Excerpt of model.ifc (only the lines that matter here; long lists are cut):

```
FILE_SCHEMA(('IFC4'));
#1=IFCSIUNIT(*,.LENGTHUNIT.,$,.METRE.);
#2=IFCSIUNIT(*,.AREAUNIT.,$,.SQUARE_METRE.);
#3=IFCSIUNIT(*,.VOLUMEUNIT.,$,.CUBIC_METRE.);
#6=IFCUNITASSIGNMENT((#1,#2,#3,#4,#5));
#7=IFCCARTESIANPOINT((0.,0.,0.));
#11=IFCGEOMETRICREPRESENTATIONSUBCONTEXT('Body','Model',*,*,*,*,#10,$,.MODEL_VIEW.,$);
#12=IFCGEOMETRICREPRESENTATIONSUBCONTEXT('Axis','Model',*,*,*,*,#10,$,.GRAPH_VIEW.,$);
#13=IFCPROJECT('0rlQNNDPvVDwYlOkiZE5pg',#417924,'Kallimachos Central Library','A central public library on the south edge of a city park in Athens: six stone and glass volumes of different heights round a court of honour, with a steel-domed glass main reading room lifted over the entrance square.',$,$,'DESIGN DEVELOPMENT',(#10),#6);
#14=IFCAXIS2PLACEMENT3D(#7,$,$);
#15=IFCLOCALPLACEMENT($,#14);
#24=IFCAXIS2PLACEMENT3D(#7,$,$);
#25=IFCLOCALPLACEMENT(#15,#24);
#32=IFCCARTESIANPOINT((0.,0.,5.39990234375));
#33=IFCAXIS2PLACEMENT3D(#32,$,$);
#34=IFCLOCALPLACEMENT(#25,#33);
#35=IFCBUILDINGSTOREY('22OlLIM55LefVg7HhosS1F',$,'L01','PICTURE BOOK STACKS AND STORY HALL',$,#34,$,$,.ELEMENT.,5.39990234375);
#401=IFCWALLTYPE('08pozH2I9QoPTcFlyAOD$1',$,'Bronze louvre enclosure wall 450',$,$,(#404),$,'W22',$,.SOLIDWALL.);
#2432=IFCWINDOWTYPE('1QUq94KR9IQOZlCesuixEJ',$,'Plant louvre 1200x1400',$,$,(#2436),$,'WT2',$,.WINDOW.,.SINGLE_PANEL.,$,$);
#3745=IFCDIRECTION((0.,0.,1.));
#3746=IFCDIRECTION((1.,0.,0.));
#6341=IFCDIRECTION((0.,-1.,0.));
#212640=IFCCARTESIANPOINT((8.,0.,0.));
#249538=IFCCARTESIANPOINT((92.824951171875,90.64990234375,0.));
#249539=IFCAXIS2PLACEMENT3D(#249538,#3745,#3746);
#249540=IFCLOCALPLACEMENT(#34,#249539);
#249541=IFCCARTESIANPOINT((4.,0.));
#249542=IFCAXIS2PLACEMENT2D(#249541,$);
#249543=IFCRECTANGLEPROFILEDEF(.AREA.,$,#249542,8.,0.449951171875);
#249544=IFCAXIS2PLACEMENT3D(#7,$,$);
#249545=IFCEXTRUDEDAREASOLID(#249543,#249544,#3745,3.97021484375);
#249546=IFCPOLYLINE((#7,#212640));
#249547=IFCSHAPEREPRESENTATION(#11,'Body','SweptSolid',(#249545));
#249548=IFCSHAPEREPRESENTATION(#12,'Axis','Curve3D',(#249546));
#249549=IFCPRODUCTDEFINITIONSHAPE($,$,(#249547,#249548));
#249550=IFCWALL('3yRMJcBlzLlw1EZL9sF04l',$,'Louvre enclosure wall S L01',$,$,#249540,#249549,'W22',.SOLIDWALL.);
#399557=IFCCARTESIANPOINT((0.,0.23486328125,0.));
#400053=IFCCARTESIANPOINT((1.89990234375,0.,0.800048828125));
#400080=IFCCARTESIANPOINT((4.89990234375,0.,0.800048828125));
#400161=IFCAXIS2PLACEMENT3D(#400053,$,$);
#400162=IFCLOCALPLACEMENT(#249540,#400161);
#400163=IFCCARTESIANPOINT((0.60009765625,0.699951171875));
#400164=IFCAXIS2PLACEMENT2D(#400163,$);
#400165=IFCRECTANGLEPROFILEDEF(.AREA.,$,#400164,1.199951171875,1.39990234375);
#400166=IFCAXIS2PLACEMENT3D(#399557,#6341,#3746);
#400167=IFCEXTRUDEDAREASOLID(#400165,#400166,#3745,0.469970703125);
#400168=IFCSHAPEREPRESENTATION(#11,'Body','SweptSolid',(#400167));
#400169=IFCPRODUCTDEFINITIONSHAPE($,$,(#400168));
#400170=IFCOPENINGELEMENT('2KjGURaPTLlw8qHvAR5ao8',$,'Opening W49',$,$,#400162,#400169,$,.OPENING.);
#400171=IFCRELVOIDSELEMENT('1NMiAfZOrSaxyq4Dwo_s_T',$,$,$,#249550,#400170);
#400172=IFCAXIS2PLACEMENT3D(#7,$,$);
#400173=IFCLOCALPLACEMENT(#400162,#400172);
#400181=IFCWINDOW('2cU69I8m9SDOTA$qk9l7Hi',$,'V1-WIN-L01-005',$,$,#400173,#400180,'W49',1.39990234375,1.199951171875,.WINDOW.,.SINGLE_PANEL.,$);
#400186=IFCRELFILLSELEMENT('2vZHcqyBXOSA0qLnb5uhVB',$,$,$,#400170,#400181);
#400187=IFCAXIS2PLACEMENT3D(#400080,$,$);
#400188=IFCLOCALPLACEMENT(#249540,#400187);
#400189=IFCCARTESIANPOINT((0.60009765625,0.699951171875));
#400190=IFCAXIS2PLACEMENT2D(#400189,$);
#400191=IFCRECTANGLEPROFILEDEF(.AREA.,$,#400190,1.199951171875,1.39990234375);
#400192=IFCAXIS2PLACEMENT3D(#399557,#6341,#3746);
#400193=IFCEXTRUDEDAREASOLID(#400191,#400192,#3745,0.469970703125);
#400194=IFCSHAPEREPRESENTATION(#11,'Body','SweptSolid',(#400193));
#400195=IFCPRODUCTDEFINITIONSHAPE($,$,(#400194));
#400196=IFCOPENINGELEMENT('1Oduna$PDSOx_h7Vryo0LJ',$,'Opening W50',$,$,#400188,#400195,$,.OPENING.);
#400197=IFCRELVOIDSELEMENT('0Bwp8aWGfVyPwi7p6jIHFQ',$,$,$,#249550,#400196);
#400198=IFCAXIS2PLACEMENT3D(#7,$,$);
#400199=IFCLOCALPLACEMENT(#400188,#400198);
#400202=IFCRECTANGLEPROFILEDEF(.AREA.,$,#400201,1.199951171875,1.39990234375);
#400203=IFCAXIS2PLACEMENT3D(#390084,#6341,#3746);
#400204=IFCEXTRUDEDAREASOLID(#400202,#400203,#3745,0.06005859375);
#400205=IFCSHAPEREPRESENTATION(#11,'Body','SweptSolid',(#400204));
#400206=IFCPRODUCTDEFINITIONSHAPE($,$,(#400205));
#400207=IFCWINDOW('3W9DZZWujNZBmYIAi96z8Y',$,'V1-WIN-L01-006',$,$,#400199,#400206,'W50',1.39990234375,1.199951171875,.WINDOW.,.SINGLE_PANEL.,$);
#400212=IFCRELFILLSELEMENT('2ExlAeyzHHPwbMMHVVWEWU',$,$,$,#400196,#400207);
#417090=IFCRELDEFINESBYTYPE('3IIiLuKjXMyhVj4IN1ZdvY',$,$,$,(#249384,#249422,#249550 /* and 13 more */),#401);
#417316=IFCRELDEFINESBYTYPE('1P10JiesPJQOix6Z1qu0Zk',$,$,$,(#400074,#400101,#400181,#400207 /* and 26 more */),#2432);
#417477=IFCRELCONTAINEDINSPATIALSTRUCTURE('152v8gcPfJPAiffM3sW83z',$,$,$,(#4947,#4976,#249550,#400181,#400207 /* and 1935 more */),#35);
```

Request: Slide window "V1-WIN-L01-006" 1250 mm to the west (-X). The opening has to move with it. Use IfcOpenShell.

```python
import ifcopenshell
import ifcopenshell.api.geometry
import ifcopenshell.util.placement
import ifcopenshell.util.unit

model = ifcopenshell.open("model.ifc")
unit_scale = ifcopenshell.util.unit.calculate_unit_scale(model)

window = model.by_guid("3W9DZZWujNZBmYIAi96z8Y")
opening = window.FillsVoids[0].RelatingOpeningElement
wall = opening.VoidsElements[0].RelatingBuildingElement

wall_matrix = ifcopenshell.util.placement.get_local_placement(wall.ObjectPlacement)
shift = wall_matrix[:3, 0] * -1.25 / unit_scale
before = ifcopenshell.util.placement.get_local_placement(window.ObjectPlacement)[:3, 3].copy()

# The window is placed relative to its opening, so it follows when the opening moves.
matrix = ifcopenshell.util.placement.get_local_placement(opening.ObjectPlacement)
matrix[:3, 3] += shift
ifcopenshell.api.geometry.edit_object_placement(
    model, product=opening, matrix=matrix, is_si=False, should_transform_children=True
)

after = ifcopenshell.util.placement.get_local_placement(window.ObjectPlacement)[:3, 3]
print("window moved by", (after - before).round(3) + 0.0)

model.write("model-out.ifc")
```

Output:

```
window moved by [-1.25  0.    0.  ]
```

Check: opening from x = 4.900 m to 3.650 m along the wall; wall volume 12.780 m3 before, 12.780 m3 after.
